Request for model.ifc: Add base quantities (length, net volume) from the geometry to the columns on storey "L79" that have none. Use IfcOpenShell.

First a look at what the model holds.

```python
import ifcopenshell
import ifcopenshell.util.element
import ifcopenshell.util.unit

model = ifcopenshell.open("model.ifc")
print(model.schema)
for unit_type in ("LENGTHUNIT", "AREAUNIT", "VOLUMEUNIT"):
    print(unit_type, ifcopenshell.util.unit.calculate_unit_scale(model, unit_type))
storey = next(s for s in model.by_type("IfcBuildingStorey") if s.Name == "L79")
columns = [e for e in ifcopenshell.util.element.get_decomposition(storey) if e.is_a("IfcColumn")]
for e in sorted(columns, key=lambda e: e.id()):
    print(e.id(), e.is_a(), e.Name, list(ifcopenshell.util.element.get_psets(e, qtos_only=True)), sep=" | ")
```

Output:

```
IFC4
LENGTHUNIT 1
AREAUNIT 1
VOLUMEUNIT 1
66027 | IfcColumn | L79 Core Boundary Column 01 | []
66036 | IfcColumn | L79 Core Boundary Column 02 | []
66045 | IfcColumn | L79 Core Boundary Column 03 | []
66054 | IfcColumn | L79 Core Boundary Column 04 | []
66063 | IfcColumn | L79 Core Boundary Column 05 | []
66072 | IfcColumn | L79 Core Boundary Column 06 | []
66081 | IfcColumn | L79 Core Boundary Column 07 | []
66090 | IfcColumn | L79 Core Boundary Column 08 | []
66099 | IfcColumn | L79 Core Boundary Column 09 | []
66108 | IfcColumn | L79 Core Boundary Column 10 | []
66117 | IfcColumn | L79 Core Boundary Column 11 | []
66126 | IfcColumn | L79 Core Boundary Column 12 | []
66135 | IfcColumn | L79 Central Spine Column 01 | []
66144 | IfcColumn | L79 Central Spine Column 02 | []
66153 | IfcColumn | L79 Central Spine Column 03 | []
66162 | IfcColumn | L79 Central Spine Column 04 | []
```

```python
import ifcopenshell
import ifcopenshell.api.pset
import ifcopenshell.geom
import ifcopenshell.util.element
import ifcopenshell.util.shape
import ifcopenshell.util.unit

model = ifcopenshell.open("model.ifc")
unit_scale = ifcopenshell.util.unit.calculate_unit_scale(model)
volume_scale = ifcopenshell.util.unit.calculate_unit_scale(model, "VOLUMEUNIT")
settings = ifcopenshell.geom.settings()

storey = next(s for s in model.by_type("IfcBuildingStorey") if s.Name == "L79")
columns = [e for e in ifcopenshell.util.element.get_decomposition(storey) if e.is_a("IfcColumn")]

for e in sorted(columns, key=lambda e: e.id()):
    if ifcopenshell.util.element.get_psets(e, qtos_only=True, should_inherit=False):
        continue
    # Geometry comes back in metres, in the element's own axes.
    shape = ifcopenshell.geom.create_shape(settings, e)
    values = {
        "Length": ifcopenshell.util.shape.get_z(shape.geometry) / unit_scale,
        "NetVolume": ifcopenshell.util.shape.get_volume(shape.geometry) / volume_scale,
    }
    qto = ifcopenshell.api.pset.add_qto(model, product=e, name="Qto_ColumnBaseQuantities")
    ifcopenshell.api.pset.edit_qto(model, qto=qto, properties=values)
    print(e.id(), {k: round(v, 3) for k, v in values.items()})

model.write("model_updated.ifc")
```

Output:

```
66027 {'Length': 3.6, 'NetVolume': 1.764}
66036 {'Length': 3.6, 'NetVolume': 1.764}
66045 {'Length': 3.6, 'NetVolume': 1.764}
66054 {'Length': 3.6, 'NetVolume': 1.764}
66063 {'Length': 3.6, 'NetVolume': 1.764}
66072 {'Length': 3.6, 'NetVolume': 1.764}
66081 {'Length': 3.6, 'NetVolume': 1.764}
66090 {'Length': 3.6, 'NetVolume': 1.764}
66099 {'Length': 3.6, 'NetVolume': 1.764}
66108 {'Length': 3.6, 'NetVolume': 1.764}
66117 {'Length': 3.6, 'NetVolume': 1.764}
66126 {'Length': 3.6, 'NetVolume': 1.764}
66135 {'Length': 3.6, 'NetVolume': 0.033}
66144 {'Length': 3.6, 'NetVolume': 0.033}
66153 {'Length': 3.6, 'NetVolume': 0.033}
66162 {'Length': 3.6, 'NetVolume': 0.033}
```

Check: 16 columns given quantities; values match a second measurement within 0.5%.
